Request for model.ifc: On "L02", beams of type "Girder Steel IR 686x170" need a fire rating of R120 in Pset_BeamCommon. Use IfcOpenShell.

First a look at what the model holds.

```python
import ifcopenshell
import ifcopenshell.util.element

model = ifcopenshell.open("model.ifc")
print(model.schema)
storey = next(s for s in model.by_type("IfcBuildingStorey") if s.Name == "L02")
beams = [e for e in ifcopenshell.util.element.get_decomposition(storey) if e.is_a("IfcBeam")]
seen = {}
for e in beams:
    element_type = ifcopenshell.util.element.get_type(e)
    key = (element_type.Name if element_type != e and element_type else None, ifcopenshell.util.element.get_pset(e, "Pset_BeamCommon", "FireRating"))
    seen[key] = seen.get(key, 0) + 1
for (name, value), count in sorted(seen.items(), key=str):
    print(count, "x", name, "|", value)
```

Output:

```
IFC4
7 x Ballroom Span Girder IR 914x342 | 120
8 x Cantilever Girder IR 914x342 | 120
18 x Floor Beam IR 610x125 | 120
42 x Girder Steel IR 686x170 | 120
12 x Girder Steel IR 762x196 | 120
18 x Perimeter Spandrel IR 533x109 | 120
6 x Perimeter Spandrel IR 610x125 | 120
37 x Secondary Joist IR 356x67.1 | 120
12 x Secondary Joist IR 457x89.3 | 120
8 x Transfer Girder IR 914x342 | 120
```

```python
import ifcopenshell
import ifcopenshell.api.pset
import ifcopenshell.util.element

model = ifcopenshell.open("model.ifc")

storey = next(s for s in model.by_type("IfcBuildingStorey") if s.Name == "L02")
beams = [e for e in ifcopenshell.util.element.get_decomposition(storey) if e.is_a("IfcBeam")]

count = 0
for e in beams:
    element_type = ifcopenshell.util.element.get_type(e)
    if element_type in (None, e) or element_type.Name != "Girder Steel IR 686x170":
        continue
    # add_pset returns the element's existing set when there is one.
    pset = ifcopenshell.api.pset.add_pset(model, product=e, name="Pset_BeamCommon")
    ifcopenshell.api.pset.edit_pset(model, pset=pset, properties={"FireRating": "R120"})
    count += 1

print(count, "beams updated")

model.write("model_rev.ifc")
```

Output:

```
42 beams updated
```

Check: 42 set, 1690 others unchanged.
